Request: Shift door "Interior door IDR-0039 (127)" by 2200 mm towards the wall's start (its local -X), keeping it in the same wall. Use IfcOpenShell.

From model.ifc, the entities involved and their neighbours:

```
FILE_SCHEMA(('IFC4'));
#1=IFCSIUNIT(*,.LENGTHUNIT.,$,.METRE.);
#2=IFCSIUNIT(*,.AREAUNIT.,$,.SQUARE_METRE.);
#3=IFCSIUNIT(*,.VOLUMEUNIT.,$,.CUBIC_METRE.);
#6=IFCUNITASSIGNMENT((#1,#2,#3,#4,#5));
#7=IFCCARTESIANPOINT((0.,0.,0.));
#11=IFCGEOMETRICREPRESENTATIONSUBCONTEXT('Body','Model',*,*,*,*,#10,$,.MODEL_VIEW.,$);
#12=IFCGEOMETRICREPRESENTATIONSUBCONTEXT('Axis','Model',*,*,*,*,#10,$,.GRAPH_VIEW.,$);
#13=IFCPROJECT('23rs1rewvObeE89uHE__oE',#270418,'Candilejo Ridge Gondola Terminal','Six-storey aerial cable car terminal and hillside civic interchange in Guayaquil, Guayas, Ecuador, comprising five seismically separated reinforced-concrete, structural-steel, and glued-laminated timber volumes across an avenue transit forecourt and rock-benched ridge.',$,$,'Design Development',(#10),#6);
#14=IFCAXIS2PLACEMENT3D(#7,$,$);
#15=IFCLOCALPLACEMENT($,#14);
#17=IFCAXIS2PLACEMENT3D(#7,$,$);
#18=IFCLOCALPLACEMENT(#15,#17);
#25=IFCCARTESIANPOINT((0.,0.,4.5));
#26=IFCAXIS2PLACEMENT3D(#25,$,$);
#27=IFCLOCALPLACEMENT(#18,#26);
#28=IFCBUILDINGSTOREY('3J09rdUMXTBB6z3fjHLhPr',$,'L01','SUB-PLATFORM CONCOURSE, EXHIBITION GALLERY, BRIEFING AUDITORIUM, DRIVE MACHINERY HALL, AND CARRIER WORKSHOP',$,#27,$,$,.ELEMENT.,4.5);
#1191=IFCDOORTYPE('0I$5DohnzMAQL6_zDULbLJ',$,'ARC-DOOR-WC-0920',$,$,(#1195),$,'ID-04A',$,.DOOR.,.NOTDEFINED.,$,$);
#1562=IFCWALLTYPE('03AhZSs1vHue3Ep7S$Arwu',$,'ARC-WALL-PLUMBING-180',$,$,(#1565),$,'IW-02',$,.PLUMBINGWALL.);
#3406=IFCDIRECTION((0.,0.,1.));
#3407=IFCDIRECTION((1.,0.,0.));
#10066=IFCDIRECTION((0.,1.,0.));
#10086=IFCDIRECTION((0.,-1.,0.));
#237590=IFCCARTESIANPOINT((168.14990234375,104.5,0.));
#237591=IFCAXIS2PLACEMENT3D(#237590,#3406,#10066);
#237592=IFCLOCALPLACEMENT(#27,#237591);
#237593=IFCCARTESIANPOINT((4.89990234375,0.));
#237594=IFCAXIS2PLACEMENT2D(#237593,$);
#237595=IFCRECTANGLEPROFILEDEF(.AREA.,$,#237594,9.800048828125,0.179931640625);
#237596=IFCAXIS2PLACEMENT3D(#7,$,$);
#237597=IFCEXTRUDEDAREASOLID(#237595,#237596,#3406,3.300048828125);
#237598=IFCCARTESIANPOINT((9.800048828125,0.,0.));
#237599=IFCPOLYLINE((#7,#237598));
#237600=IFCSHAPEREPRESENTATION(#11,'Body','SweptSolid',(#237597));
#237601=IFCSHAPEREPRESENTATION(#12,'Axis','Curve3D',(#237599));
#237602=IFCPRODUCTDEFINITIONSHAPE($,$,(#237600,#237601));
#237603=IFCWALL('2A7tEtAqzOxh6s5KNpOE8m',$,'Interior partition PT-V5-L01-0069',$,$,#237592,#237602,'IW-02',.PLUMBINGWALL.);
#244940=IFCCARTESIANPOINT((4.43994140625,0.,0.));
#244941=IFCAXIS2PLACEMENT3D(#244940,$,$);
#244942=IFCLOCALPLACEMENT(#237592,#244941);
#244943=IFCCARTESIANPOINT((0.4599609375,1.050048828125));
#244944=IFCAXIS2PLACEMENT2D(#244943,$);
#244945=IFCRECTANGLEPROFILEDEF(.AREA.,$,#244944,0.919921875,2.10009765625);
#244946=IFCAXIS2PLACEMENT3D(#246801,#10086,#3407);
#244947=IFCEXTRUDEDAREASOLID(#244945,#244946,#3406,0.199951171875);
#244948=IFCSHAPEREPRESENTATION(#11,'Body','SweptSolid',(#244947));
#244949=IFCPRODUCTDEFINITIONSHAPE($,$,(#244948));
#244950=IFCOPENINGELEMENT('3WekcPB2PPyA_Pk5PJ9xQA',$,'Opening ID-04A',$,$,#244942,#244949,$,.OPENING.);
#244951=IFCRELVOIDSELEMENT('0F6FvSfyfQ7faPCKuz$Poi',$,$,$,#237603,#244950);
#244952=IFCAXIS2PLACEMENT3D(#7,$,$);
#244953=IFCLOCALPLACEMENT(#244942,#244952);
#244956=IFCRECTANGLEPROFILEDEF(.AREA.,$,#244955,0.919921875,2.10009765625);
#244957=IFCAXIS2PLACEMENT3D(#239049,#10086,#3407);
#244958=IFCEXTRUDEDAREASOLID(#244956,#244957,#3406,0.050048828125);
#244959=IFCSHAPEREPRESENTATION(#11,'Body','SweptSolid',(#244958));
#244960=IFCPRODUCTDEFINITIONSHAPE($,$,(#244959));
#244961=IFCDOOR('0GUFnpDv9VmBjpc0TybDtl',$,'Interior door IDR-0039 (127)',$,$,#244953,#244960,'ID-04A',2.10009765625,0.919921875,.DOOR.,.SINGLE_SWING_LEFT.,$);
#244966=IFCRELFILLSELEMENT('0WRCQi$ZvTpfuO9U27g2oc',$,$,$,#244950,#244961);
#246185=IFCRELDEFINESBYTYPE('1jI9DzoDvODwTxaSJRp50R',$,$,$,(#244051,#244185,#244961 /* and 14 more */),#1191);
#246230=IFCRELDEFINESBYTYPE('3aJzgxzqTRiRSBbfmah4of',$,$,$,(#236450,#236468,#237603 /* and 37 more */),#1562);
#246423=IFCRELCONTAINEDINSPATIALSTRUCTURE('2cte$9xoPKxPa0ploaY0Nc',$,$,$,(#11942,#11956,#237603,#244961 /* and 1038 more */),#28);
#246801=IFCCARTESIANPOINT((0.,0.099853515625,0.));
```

```python
import ifcopenshell
import ifcopenshell.api.geometry
import ifcopenshell.util.placement

model = ifcopenshell.open("model.ifc")

door = model.by_id(244961)
opening = door.FillsVoids[0].RelatingOpeningElement
wall = opening.VoidsElements[0].RelatingBuildingElement

wall_matrix = ifcopenshell.util.placement.get_local_placement(wall.ObjectPlacement)
shift = wall_matrix[:3, 0] * -2.2
before = ifcopenshell.util.placement.get_local_placement(door.ObjectPlacement)[:3, 3].copy()

# The door is placed relative to its opening, so it follows when the opening moves.
matrix = ifcopenshell.util.placement.get_local_placement(opening.ObjectPlacement)
matrix[:3, 3] += shift
ifcopenshell.api.geometry.edit_object_placement(
    model, product=opening, matrix=matrix, is_si=False, should_transform_children=True
)

after = ifcopenshell.util.placement.get_local_placement(door.ObjectPlacement)[:3, 3]
print("door moved by", (after - before).round(3) + 0.0)

model.write("model_updated.ifc")
```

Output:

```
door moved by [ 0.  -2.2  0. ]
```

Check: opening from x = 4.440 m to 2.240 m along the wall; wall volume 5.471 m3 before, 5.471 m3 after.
